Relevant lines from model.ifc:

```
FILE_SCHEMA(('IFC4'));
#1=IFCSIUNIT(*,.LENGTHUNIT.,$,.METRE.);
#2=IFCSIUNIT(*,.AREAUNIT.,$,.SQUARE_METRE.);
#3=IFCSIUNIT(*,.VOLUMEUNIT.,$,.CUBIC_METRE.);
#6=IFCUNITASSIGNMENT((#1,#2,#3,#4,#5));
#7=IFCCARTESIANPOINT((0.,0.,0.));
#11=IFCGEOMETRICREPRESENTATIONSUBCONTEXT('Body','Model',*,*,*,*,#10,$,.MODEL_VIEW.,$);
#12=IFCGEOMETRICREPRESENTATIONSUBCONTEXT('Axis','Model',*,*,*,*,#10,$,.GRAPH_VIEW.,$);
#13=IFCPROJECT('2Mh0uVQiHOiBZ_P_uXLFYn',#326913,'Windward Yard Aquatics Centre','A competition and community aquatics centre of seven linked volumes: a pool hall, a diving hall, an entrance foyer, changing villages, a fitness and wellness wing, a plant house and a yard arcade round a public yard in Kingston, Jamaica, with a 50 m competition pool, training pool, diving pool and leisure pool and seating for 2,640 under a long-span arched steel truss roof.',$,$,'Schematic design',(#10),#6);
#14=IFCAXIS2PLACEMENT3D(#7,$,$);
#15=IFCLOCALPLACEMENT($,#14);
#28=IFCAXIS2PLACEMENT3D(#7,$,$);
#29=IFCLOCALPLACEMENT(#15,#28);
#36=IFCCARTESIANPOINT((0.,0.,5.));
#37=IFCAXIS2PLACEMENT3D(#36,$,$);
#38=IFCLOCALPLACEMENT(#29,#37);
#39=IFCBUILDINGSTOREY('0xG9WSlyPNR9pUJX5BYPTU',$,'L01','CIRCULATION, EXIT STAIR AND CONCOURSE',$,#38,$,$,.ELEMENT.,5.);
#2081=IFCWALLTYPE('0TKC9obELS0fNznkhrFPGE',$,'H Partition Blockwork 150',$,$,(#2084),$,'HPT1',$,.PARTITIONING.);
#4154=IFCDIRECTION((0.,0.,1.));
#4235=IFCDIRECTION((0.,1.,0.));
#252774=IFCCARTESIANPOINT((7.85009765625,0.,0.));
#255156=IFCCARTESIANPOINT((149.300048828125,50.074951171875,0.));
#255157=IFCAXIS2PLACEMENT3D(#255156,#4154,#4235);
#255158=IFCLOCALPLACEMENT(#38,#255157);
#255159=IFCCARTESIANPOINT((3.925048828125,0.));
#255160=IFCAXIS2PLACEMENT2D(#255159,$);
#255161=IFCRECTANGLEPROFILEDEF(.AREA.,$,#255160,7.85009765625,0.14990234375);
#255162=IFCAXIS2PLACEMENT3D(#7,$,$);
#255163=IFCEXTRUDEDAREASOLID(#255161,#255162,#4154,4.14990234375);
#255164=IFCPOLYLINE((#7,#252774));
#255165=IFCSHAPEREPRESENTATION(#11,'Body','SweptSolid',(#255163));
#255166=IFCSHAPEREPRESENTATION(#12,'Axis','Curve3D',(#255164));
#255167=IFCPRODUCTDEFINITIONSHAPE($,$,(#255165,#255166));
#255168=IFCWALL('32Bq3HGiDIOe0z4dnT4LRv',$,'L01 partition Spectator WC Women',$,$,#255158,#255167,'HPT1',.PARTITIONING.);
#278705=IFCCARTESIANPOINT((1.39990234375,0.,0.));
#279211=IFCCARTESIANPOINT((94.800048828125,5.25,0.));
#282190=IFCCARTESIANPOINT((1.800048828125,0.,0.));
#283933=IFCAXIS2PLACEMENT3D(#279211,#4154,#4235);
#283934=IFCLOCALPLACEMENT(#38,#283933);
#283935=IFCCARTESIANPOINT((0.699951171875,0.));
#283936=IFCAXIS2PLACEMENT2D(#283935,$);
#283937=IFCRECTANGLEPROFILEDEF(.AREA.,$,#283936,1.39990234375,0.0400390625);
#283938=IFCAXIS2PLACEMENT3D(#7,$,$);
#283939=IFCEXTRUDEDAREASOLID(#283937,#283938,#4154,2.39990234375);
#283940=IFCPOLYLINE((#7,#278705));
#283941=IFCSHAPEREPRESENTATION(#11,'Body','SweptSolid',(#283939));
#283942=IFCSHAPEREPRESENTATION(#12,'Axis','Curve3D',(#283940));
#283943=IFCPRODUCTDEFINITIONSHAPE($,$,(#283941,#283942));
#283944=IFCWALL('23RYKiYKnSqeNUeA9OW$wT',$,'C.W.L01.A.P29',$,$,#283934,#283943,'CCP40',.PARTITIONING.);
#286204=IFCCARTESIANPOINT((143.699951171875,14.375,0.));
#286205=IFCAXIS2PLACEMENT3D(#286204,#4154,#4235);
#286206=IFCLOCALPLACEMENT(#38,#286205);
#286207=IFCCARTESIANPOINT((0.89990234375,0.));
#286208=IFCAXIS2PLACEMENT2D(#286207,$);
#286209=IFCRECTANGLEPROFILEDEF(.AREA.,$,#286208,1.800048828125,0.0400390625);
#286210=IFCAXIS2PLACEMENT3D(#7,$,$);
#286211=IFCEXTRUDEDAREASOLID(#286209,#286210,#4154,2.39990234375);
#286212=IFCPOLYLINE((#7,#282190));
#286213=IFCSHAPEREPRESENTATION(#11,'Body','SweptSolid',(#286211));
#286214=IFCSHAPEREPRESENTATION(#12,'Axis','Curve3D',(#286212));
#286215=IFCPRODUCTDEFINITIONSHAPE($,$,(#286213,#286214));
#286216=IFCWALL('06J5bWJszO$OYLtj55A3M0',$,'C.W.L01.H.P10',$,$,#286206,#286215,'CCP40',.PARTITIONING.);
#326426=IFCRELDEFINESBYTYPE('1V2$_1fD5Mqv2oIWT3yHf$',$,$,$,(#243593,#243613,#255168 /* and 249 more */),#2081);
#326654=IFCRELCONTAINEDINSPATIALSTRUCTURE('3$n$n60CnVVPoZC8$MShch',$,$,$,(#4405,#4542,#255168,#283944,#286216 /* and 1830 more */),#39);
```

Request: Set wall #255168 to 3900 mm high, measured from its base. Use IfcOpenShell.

```python
import ifcopenshell
import ifcopenshell.geom
import ifcopenshell.util.representation
import ifcopenshell.util.shape

model = ifcopenshell.open("model.ifc")
settings = ifcopenshell.geom.settings()


def volume(element):
    """Net volume in cubic metres, openings subtracted."""
    shape = ifcopenshell.geom.create_shape(settings, element)
    return ifcopenshell.util.shape.get_volume(shape.geometry)


wall = model.by_id(255168)
before = volume(wall)

body = ifcopenshell.util.representation.get_representation(wall, "Model", "Body")
solid = body.Items[0]
old_height = solid.Depth
solid.Depth = 3.9
after = volume(wall)

print(f"height {old_height:g} -> {solid.Depth:g}, volume {before:.3f} -> {after:.3f} m3")

model.write("model-out.ifc")
```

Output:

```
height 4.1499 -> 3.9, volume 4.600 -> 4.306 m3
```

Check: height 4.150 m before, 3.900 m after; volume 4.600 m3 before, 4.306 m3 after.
